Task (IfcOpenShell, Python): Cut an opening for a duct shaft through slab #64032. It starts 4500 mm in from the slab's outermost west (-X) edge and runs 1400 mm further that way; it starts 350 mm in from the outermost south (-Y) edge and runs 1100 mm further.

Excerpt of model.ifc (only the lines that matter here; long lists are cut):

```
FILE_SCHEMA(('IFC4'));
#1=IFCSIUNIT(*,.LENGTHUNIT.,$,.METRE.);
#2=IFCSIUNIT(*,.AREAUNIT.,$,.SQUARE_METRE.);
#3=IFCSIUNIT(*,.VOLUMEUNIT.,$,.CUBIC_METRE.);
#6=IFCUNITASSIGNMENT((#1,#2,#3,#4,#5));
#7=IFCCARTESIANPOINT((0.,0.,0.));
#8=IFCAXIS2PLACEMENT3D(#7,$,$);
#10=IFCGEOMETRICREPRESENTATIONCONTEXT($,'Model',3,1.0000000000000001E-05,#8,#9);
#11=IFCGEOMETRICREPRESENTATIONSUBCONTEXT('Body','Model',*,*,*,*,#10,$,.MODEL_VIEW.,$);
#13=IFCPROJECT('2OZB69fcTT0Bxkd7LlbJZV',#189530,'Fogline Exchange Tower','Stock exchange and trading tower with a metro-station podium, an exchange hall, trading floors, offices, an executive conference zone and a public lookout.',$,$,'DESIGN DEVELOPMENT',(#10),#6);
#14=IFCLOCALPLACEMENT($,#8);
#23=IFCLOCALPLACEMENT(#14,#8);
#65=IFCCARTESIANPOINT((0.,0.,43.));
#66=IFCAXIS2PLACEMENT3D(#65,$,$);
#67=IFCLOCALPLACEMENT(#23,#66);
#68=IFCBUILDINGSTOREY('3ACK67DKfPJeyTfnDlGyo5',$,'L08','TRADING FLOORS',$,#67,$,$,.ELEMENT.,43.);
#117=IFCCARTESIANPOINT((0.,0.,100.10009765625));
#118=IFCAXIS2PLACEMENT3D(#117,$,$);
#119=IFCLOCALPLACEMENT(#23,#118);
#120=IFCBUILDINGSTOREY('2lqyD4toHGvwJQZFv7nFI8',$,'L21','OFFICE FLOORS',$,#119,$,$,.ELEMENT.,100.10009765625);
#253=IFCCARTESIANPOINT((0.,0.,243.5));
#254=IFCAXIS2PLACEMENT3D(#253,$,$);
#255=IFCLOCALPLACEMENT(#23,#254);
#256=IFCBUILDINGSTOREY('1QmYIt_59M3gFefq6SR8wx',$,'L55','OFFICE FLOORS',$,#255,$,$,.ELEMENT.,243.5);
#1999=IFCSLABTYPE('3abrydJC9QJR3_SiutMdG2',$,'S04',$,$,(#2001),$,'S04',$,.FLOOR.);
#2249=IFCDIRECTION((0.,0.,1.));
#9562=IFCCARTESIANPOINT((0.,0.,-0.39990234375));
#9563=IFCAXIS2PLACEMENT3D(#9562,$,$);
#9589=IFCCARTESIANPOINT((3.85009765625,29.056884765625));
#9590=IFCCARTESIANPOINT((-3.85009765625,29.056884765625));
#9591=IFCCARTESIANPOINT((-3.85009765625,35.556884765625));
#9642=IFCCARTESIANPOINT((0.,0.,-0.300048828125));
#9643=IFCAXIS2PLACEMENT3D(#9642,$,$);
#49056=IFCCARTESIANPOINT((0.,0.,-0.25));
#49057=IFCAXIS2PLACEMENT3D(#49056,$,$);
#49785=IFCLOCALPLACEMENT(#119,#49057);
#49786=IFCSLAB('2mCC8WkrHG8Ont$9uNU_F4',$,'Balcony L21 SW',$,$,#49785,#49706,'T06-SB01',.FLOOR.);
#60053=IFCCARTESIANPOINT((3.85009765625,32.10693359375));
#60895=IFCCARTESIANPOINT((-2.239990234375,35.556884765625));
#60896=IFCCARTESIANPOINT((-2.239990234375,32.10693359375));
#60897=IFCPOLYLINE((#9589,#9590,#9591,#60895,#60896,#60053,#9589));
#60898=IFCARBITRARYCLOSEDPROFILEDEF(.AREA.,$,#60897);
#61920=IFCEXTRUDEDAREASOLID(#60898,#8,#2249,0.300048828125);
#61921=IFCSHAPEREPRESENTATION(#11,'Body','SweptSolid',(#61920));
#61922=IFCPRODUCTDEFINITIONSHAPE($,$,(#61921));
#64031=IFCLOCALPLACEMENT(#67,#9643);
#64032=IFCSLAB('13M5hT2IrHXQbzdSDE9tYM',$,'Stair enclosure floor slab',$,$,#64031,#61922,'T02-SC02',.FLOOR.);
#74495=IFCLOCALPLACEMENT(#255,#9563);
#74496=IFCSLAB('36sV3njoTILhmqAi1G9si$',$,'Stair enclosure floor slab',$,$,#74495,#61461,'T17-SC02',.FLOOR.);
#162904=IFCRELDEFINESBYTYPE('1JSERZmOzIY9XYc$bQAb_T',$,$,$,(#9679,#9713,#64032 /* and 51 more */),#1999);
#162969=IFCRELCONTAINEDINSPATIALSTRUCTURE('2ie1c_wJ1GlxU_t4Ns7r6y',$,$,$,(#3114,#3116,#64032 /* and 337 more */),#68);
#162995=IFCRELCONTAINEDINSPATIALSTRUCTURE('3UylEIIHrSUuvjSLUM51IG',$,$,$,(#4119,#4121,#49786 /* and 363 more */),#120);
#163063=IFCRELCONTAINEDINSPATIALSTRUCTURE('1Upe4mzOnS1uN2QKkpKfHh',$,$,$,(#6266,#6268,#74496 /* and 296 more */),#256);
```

```python
import numpy as np
import ifcopenshell
import ifcopenshell.api.feature
import ifcopenshell.api.geometry
import ifcopenshell.api.root
import ifcopenshell.geom
import ifcopenshell.util.placement
import ifcopenshell.util.representation
import ifcopenshell.util.shape
import ifcopenshell.util.unit

model = ifcopenshell.open("model.ifc")
unit_scale = ifcopenshell.util.unit.calculate_unit_scale(model)
settings = ifcopenshell.geom.settings()


def volume(element):
    """Net volume in cubic metres, openings subtracted."""
    shape = ifcopenshell.geom.create_shape(settings, element)
    return ifcopenshell.util.shape.get_volume(shape.geometry)


slab = model.by_guid("13M5hT2IrHXQbzdSDE9tYM")
before = volume(slab)

# Extent in the slab's own axes, in metres. The edges named are its -X and -Y sides.
slab_shape = ifcopenshell.geom.create_shape(settings, slab)
vertices = ifcopenshell.util.shape.get_vertices(slab_shape.geometry)
x_min, y_min, bottom = vertices.min(axis=0)
top = vertices[:, 2].max()

opening = ifcopenshell.api.root.create_entity(model, ifc_class="IfcOpeningElement", name="Duct shaft opening", predefined_type="OPENING")
context = ifcopenshell.util.representation.get_context(model, "Model", "Body", "MODEL_VIEW")
width, depth = 1.4, 1.1
outline = [(0.0, 0.0), (width, 0.0), (width, depth), (0.0, depth), (0.0, 0.0)]
# Overshoot both faces by 50 mm so the cut is clean.
shape = ifcopenshell.api.geometry.add_slab_representation(
    model, context=context, depth=top - bottom + 0.1, polyline=outline
)
ifcopenshell.api.geometry.assign_representation(model, product=opening, representation=shape)

matrix = ifcopenshell.util.placement.get_local_placement(slab.ObjectPlacement)
matrix[:, 3] = matrix @ np.append(np.array([x_min + 4.5, y_min + 0.35, bottom - 0.05]) / unit_scale, 1.0)
ifcopenshell.api.geometry.edit_object_placement(model, product=opening, matrix=matrix, is_si=False)
ifcopenshell.api.feature.add_feature(model, feature=opening, element=slab)

after = volume(slab)

print(f"slab volume {before:.3f} -> {after:.3f} m3")

model.write("model-out.ifc")
```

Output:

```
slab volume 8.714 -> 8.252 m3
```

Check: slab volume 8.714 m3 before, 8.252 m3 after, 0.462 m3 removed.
